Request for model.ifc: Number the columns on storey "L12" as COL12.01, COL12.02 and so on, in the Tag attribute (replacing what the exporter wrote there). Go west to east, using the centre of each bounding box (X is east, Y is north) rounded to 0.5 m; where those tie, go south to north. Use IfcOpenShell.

First a look at what the model holds.

```python
import ifcopenshell
import ifcopenshell.util.element
import ifcopenshell.util.placement

model = ifcopenshell.open("model.ifc")
print(model.schema)
storey = next(s for s in model.by_type("IfcBuildingStorey") if s.Name == "L12")
columns = [e for e in ifcopenshell.util.element.get_decomposition(storey) if e.is_a("IfcColumn")]
for e in sorted(columns, key=lambda e: e.id()):
    origin = ifcopenshell.util.placement.get_local_placement(e.ObjectPlacement)[:3, 3]
    print(e.id(), e.Tag, e.Name, origin.round(2) + 0.0, sep=" | ")
```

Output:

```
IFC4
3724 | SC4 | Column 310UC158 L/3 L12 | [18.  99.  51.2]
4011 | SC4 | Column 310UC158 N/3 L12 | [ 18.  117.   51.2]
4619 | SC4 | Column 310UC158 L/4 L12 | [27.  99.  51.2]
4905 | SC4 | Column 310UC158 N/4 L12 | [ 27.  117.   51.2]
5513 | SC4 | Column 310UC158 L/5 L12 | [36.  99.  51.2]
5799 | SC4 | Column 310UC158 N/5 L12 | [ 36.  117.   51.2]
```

```python
import ifcopenshell
import ifcopenshell.geom
import ifcopenshell.util.element
import ifcopenshell.util.shape

model = ifcopenshell.open("model.ifc")
settings = ifcopenshell.geom.settings()
settings.set("use-world-coords", True)


def centre(element):
    shape = ifcopenshell.geom.create_shape(settings, element)
    return ifcopenshell.util.shape.get_bbox_centroid(shape.geometry)


storey = next(s for s in model.by_type("IfcBuildingStorey") if s.Name == "L12")
columns = [e for e in ifcopenshell.util.element.get_decomposition(storey) if e.is_a("IfcColumn")]

# Insertion points can sit at a corner or the storey origin, so sort by the geometry (in metres).
centres = {e: centre(e) for e in columns}
columns.sort(key=lambda e: (round(centres[e][0] / 0.5), centres[e][1]))

for i, e in enumerate(columns, start=1):
    number = f"COL12.{i:02d}"
    e.Tag = number
    print(e.id(), number)

model.write("model_updated.ifc")
```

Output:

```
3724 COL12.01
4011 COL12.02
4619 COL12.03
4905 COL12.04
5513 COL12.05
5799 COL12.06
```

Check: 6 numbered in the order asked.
